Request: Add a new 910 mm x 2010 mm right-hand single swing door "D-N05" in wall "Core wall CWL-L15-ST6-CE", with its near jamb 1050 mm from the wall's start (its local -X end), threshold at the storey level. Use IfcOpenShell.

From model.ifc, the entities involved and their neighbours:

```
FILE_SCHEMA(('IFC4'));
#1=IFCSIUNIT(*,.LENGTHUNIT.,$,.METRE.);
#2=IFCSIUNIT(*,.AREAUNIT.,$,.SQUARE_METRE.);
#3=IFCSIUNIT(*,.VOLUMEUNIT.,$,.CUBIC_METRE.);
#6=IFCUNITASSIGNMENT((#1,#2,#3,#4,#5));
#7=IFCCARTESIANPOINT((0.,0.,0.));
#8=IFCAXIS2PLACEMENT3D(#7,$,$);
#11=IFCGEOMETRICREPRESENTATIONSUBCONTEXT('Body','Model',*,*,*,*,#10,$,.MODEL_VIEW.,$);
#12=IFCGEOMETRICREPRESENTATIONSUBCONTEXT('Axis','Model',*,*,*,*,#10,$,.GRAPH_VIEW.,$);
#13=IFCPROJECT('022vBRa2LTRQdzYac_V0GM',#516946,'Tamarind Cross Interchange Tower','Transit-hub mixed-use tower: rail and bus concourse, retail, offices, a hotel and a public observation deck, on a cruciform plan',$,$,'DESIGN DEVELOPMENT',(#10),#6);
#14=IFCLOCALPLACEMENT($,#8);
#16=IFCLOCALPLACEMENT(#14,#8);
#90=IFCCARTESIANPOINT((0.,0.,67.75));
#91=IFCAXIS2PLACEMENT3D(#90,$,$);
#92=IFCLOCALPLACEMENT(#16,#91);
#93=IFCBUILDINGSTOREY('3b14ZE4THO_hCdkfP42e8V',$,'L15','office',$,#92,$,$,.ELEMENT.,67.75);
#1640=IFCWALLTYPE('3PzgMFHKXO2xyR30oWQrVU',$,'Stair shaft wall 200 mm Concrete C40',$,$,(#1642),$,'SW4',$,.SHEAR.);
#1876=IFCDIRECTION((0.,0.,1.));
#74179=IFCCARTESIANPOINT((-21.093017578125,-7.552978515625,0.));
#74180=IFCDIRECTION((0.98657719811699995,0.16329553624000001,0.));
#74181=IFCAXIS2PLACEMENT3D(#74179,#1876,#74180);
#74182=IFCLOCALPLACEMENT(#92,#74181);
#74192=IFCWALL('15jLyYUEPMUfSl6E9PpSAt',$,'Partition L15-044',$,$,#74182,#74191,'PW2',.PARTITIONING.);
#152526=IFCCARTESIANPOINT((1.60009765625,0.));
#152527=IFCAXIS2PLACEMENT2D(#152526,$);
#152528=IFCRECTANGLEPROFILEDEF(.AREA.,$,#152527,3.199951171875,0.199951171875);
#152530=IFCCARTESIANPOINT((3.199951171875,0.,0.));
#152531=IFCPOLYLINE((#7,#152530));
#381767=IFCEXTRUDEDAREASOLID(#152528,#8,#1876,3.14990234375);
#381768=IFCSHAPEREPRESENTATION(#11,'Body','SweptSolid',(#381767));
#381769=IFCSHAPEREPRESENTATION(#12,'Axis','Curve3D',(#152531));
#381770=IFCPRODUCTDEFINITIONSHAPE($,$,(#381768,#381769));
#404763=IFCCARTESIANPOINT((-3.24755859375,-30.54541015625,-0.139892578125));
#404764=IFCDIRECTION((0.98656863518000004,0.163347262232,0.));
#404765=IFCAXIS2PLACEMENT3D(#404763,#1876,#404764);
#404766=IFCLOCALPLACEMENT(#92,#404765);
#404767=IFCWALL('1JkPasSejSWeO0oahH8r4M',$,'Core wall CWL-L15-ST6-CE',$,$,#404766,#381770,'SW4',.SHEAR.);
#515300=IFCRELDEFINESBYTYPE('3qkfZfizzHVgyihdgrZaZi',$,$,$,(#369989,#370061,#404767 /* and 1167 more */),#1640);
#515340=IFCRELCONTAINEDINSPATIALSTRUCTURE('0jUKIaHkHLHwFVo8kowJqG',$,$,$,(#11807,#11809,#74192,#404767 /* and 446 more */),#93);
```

```python
import numpy as np
import ifcopenshell
import ifcopenshell.api.feature
import ifcopenshell.api.geometry
import ifcopenshell.api.root
import ifcopenshell.api.spatial
import ifcopenshell.geom
import ifcopenshell.util.element
import ifcopenshell.util.placement
import ifcopenshell.util.representation
import ifcopenshell.util.shape
import ifcopenshell.util.unit

model = ifcopenshell.open("model.ifc")
unit_scale = ifcopenshell.util.unit.calculate_unit_scale(model)
settings = ifcopenshell.geom.settings()


def volume(element):
    """Net volume in cubic metres, openings subtracted."""
    shape = ifcopenshell.geom.create_shape(settings, element)
    return ifcopenshell.util.shape.get_volume(shape.geometry)


wall = model.by_guid("1JkPasSejSWeO0oahH8r4M")
storey = ifcopenshell.util.element.get_container(wall, ifc_class="IfcBuildingStorey")
context = ifcopenshell.util.representation.get_context(model, "Model", "Body", "MODEL_VIEW")
before = volume(wall)

width, height, from_end, sill = 0.91, 2.01, 1.05, 0.0  # metres

# The wall runs along its own X axis, and the end named is its -X end.
wall_shape = ifcopenshell.geom.create_shape(settings, wall)
x, y, z = ifcopenshell.util.shape.get_vertices(wall_shape.geometry).T
start = x.min() + from_end
face, thickness = float(y.min()), float(y.max() - y.min())
wall_matrix = ifcopenshell.util.placement.get_local_placement(wall.ObjectPlacement)
level = ifcopenshell.util.placement.get_local_placement(storey.ObjectPlacement)[2, 3]


def in_wall(x, y):
    """Placement at x, y metres in the wall's axes, at sill height."""
    matrix = wall_matrix.copy()
    matrix[:, 3] = wall_matrix @ np.array([x / unit_scale, y / unit_scale, 0.0, 1.0])
    matrix[2, 3] = level + sill / unit_scale
    return matrix


# Opening: a box that overshoots both wall faces by 50 mm.
opening = ifcopenshell.api.root.create_entity(model, ifc_class="IfcOpeningElement", predefined_type="OPENING")
box = ifcopenshell.api.geometry.add_wall_representation(
    model, context=context, length=width, height=height, thickness=thickness + 0.1
)
ifcopenshell.api.geometry.assign_representation(model, product=opening, representation=box)
ifcopenshell.api.geometry.edit_object_placement(model, product=opening, matrix=in_wall(start, face - 0.05), is_si=False)
ifcopenshell.api.feature.add_feature(model, feature=opening, element=wall)

door = ifcopenshell.api.root.create_entity(model, ifc_class="IfcDoor", name="D-N05", predefined_type="DOOR")
door.OverallWidth, door.OverallHeight = width / unit_scale, height / unit_scale
door.OperationType = "SINGLE_SWING_RIGHT"
body = ifcopenshell.api.geometry.add_door_representation(
    model,
    context=context,
    overall_width=door.OverallWidth,
    overall_height=door.OverallHeight,
    operation_type="SINGLE_SWING_RIGHT",
    lining_properties={"LiningDepth": thickness / unit_scale, "ThresholdDepth": thickness / unit_scale},
)
ifcopenshell.api.geometry.assign_representation(model, product=door, representation=body)
ifcopenshell.api.spatial.assign_container(model, products=[door], relating_structure=storey)
ifcopenshell.api.feature.add_filling(model, opening=opening, element=door)

# The lining spans the wall, so the door starts at the wall face.
ifcopenshell.api.geometry.edit_object_placement(model, product=door, matrix=in_wall(start, face), is_si=False)

after = volume(wall)

print(f"wall volume {before:.3f} -> {after:.3f} m3")

model.write("model_edited.ifc")
```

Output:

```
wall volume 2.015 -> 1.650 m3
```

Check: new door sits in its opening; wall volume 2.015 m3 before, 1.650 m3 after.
